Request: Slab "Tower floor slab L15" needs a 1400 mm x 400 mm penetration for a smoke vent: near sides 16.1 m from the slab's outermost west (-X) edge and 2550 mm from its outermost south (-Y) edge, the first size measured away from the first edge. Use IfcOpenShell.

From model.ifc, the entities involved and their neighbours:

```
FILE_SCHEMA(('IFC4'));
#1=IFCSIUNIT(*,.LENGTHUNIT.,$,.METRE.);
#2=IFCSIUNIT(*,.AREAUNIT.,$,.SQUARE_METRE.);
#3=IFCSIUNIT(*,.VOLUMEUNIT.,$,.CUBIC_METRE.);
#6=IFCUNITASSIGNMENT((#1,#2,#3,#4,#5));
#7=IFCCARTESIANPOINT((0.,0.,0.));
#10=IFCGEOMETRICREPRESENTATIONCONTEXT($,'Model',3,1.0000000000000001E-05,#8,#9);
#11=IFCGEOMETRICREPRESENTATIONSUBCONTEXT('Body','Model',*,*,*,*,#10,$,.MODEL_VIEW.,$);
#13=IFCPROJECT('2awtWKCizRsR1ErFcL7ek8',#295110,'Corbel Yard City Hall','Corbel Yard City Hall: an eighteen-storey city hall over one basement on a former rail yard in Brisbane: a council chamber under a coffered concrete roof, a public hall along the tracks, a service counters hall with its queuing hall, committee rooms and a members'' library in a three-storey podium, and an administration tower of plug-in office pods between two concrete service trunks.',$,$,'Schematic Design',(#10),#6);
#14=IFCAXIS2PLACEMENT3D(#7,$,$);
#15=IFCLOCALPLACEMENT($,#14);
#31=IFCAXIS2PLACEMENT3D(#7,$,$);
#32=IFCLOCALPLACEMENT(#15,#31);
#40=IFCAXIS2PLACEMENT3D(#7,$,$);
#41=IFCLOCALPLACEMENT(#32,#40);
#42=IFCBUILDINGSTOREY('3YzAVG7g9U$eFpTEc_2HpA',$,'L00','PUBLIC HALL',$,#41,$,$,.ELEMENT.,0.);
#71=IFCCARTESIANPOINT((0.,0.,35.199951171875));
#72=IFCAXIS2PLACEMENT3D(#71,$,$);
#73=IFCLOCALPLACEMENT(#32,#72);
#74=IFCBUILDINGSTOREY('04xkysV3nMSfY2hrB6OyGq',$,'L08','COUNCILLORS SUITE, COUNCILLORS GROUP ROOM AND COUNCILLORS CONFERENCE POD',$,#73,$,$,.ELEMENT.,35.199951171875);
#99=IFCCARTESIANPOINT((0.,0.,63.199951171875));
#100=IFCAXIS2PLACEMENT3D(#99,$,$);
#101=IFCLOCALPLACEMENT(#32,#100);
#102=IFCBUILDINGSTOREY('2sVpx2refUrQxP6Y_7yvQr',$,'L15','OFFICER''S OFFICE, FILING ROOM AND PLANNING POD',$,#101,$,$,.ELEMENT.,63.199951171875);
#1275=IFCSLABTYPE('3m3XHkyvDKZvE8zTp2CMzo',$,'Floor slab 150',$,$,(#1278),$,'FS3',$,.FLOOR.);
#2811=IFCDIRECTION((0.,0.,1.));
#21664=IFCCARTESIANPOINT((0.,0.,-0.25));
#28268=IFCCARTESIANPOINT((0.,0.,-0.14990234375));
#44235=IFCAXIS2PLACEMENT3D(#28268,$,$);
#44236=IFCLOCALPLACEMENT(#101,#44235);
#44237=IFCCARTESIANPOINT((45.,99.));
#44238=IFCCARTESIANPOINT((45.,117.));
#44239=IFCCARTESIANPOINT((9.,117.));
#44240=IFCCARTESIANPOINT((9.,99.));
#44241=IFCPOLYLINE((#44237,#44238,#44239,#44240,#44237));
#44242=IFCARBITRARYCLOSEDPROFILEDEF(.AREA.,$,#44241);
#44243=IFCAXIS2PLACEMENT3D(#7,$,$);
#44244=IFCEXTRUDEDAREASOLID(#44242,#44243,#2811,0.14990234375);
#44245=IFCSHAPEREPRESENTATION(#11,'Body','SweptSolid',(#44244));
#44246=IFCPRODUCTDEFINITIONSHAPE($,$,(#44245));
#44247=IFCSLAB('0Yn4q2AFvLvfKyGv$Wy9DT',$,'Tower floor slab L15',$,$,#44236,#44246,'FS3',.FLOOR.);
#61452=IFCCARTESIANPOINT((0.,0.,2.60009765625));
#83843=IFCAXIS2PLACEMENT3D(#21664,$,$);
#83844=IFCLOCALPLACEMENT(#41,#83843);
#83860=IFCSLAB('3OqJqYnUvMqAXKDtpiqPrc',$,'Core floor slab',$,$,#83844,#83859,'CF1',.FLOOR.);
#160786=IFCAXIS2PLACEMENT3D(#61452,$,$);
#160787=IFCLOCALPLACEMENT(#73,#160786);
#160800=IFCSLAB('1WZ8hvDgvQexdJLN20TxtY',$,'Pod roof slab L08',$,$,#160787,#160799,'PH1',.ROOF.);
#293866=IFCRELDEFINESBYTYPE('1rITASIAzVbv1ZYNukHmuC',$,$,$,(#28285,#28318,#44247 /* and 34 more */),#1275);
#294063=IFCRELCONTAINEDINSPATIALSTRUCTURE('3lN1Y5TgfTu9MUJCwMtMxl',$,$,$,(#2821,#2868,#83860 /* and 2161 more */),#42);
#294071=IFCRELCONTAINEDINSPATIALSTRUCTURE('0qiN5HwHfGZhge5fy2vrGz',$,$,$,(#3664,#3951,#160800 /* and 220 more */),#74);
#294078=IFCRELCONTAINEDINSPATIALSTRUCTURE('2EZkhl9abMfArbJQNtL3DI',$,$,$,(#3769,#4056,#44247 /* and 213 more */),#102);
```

```python
import numpy as np
import ifcopenshell
import ifcopenshell.api.feature
import ifcopenshell.api.geometry
import ifcopenshell.api.root
import ifcopenshell.geom
import ifcopenshell.util.placement
import ifcopenshell.util.representation
import ifcopenshell.util.shape
import ifcopenshell.util.unit

model = ifcopenshell.open("model.ifc")
unit_scale = ifcopenshell.util.unit.calculate_unit_scale(model)
settings = ifcopenshell.geom.settings()


def volume(element):
    """Net volume in cubic metres, openings subtracted."""
    shape = ifcopenshell.geom.create_shape(settings, element)
    return ifcopenshell.util.shape.get_volume(shape.geometry)


slab = model.by_guid("0Yn4q2AFvLvfKyGv$Wy9DT")
before = volume(slab)

# Extent in the slab's own axes, in metres. The edges named are its -X and -Y sides.
slab_shape = ifcopenshell.geom.create_shape(settings, slab)
vertices = ifcopenshell.util.shape.get_vertices(slab_shape.geometry)
x_min, y_min, bottom = vertices.min(axis=0)
top = vertices[:, 2].max()

opening = ifcopenshell.api.root.create_entity(model, ifc_class="IfcOpeningElement", name="Smoke vent opening", predefined_type="OPENING")
context = ifcopenshell.util.representation.get_context(model, "Model", "Body", "MODEL_VIEW")
width, depth = 1.4, 0.4
outline = [(0.0, 0.0), (width, 0.0), (width, depth), (0.0, depth), (0.0, 0.0)]
# Overshoot both faces by 50 mm so the cut is clean.
shape = ifcopenshell.api.geometry.add_slab_representation(
    model, context=context, depth=top - bottom + 0.1, polyline=outline
)
ifcopenshell.api.geometry.assign_representation(model, product=opening, representation=shape)

matrix = ifcopenshell.util.placement.get_local_placement(slab.ObjectPlacement)
matrix[:, 3] = matrix @ np.append(np.array([x_min + 16.1, y_min + 2.55, bottom - 0.05]) / unit_scale, 1.0)
ifcopenshell.api.geometry.edit_object_placement(model, product=opening, matrix=matrix, is_si=False)
ifcopenshell.api.feature.add_feature(model, feature=opening, element=slab)

after = volume(slab)

print(f"slab volume {before:.3f} -> {after:.3f} m3")

model.write("model-out.ifc")
```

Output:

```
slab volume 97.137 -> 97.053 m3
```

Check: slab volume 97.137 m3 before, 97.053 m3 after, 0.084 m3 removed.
